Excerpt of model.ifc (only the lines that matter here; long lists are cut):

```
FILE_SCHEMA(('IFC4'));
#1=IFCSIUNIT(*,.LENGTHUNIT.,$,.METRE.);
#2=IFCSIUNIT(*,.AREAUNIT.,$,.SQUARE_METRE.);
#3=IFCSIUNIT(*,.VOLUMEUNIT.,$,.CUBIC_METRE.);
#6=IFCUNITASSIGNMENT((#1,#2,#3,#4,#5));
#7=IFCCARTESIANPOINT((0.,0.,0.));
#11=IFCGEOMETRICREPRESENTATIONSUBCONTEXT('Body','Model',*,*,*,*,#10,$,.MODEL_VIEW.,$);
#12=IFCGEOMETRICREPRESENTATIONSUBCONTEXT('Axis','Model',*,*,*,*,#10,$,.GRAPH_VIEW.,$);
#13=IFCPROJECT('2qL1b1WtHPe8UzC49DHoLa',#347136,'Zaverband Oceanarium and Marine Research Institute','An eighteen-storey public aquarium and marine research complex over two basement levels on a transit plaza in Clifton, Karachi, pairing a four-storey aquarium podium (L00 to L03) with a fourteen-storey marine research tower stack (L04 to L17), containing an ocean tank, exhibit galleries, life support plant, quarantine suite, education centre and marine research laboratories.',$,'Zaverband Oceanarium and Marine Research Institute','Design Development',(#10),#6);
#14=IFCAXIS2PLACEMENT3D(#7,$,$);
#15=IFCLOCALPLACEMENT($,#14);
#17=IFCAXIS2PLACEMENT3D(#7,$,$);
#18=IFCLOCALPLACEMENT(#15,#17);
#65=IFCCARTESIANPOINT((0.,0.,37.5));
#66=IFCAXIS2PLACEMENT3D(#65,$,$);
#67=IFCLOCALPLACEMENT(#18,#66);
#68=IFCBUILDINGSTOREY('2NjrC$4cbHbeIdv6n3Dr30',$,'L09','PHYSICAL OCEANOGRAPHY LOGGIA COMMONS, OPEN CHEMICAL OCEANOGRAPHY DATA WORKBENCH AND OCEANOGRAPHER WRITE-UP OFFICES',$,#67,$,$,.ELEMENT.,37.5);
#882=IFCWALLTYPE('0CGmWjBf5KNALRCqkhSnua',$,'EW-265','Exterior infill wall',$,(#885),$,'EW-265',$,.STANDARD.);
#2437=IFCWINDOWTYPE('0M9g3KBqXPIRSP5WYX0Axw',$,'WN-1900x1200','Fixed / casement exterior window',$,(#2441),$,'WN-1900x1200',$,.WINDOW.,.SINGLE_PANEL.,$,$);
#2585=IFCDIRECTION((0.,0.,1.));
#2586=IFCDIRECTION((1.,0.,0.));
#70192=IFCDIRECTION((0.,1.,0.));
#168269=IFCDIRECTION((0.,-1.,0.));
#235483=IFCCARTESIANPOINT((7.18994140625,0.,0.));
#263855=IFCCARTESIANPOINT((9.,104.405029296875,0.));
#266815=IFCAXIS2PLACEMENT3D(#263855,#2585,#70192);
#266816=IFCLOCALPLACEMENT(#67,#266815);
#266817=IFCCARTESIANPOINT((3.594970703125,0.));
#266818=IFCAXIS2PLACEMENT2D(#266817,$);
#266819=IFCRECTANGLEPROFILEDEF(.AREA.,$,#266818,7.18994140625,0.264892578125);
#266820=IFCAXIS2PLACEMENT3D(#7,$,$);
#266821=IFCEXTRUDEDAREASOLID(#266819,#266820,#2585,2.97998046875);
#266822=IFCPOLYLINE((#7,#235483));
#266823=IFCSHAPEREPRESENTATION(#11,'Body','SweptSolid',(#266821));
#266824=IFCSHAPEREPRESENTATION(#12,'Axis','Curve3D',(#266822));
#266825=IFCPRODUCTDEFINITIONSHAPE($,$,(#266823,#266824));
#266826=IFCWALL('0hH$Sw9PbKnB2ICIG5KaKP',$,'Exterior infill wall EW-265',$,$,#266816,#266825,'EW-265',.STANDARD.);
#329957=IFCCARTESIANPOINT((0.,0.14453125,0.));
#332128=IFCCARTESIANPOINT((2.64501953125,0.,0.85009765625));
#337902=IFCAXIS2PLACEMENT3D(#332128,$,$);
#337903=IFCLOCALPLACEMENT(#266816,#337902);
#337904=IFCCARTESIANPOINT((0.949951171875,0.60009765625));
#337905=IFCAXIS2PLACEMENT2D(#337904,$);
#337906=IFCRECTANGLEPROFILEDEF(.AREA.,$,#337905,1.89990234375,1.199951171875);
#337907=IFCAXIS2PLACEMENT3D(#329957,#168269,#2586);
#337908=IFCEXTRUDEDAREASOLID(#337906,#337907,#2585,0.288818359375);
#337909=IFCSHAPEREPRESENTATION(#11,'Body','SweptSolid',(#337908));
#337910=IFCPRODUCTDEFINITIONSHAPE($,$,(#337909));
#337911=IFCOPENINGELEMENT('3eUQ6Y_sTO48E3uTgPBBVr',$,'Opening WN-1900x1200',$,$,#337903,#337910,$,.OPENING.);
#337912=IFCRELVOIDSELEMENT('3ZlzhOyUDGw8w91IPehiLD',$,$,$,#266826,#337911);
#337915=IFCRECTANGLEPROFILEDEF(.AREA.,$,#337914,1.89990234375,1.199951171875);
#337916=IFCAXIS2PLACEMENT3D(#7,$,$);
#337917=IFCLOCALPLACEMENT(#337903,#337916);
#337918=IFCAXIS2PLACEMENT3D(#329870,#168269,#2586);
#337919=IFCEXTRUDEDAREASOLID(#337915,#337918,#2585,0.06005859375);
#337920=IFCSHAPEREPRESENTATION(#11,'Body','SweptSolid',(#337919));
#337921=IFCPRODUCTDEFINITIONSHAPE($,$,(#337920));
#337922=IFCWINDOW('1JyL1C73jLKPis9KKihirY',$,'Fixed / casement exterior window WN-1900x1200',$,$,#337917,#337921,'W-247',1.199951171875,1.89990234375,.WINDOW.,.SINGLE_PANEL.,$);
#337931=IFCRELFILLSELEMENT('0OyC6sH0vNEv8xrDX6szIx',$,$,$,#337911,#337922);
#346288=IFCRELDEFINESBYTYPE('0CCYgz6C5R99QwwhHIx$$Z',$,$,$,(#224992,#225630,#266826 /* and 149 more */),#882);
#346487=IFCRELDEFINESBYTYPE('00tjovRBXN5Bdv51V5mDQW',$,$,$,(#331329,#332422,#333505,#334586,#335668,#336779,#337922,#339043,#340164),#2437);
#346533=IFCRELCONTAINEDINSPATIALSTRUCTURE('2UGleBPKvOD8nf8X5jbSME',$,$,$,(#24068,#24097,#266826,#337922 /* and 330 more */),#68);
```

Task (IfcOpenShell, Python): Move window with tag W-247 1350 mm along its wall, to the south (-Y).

```python
import ifcopenshell
import ifcopenshell.api.geometry
import ifcopenshell.util.placement

model = ifcopenshell.open("model.ifc")

window = model.by_id(337922)
opening = window.FillsVoids[0].RelatingOpeningElement
wall = opening.VoidsElements[0].RelatingBuildingElement

wall_matrix = ifcopenshell.util.placement.get_local_placement(wall.ObjectPlacement)
shift = wall_matrix[:3, 0] * -1.35
before = ifcopenshell.util.placement.get_local_placement(window.ObjectPlacement)[:3, 3].copy()

# The window is placed relative to its opening, so it follows when the opening moves.
matrix = ifcopenshell.util.placement.get_local_placement(opening.ObjectPlacement)
matrix[:3, 3] += shift
ifcopenshell.api.geometry.edit_object_placement(
    model, product=opening, matrix=matrix, is_si=False, should_transform_children=True
)

after = ifcopenshell.util.placement.get_local_placement(window.ObjectPlacement)[:3, 3]
print("window moved by", (after - before).round(3) + 0.0)

model.write("model_rev.ifc")
```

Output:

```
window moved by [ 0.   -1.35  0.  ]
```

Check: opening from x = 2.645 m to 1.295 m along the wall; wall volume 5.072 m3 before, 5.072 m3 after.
